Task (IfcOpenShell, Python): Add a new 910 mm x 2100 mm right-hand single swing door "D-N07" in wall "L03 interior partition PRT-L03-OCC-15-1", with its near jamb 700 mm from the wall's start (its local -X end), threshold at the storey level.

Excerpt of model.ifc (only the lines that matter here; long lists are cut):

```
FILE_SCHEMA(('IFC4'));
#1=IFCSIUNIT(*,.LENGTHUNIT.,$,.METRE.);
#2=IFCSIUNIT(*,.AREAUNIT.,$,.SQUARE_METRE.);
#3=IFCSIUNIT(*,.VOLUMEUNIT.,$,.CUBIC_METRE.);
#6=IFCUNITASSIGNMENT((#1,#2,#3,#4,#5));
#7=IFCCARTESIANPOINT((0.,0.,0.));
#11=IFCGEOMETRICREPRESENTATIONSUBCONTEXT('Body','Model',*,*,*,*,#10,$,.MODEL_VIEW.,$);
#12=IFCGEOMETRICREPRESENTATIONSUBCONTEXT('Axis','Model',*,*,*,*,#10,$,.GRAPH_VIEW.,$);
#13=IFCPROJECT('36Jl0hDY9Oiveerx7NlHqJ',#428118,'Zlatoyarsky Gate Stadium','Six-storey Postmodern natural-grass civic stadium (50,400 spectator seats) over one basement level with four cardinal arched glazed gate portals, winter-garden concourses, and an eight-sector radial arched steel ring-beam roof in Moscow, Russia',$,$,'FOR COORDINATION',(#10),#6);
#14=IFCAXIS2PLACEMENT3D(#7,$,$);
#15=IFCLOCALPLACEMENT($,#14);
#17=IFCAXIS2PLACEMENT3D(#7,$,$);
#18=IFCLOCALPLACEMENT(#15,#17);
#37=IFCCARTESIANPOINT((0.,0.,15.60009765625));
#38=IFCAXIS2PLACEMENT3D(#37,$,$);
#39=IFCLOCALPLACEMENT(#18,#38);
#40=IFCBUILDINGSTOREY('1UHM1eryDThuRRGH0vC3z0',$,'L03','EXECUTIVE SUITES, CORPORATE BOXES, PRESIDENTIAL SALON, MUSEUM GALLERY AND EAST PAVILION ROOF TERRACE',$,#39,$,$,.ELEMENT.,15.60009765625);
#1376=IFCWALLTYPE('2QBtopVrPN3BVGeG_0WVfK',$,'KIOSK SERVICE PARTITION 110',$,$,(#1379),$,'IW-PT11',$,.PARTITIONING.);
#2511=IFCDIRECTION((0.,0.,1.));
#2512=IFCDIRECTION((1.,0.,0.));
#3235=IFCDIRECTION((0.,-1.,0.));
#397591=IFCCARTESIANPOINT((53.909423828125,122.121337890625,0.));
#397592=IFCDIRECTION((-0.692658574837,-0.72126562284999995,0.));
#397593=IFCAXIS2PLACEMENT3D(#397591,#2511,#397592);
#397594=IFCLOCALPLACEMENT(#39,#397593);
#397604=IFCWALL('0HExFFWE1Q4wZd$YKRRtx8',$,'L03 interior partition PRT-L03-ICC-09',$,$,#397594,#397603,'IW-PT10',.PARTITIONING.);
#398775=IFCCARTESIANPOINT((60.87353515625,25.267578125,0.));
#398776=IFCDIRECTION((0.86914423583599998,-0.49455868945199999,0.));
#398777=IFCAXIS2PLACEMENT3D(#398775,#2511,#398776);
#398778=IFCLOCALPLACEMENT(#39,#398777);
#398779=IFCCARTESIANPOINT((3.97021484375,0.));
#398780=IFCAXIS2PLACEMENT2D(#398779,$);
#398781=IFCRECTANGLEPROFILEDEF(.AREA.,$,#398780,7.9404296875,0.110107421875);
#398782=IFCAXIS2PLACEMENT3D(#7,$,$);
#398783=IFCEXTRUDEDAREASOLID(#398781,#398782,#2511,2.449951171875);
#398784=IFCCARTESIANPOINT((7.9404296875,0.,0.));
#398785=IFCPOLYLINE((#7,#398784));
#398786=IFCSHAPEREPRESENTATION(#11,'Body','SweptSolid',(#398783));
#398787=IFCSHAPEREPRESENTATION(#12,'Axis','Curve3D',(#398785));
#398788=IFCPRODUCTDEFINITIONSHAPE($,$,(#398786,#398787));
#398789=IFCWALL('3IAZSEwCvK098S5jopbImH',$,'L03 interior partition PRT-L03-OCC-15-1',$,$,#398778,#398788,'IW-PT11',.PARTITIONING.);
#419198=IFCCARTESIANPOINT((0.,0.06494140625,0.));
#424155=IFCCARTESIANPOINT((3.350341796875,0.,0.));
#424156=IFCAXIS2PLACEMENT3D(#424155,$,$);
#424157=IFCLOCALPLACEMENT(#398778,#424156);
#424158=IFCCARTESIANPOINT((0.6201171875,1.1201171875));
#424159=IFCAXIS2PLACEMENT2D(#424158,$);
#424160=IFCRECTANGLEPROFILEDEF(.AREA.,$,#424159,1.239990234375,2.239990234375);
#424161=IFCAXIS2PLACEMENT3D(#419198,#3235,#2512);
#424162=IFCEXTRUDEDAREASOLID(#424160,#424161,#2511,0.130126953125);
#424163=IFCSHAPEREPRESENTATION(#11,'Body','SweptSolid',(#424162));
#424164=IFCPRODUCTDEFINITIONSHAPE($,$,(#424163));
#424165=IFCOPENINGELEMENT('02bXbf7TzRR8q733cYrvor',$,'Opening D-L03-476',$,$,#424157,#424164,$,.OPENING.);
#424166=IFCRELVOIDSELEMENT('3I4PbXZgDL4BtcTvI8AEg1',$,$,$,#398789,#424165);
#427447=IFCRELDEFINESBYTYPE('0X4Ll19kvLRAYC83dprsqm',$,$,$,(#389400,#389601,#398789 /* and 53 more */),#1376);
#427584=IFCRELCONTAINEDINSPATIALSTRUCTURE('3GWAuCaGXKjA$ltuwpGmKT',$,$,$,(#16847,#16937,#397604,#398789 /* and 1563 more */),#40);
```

```python
import numpy as np
import ifcopenshell
import ifcopenshell.api.feature
import ifcopenshell.api.geometry
import ifcopenshell.api.root
import ifcopenshell.api.spatial
import ifcopenshell.geom
import ifcopenshell.util.element
import ifcopenshell.util.placement
import ifcopenshell.util.representation
import ifcopenshell.util.shape
import ifcopenshell.util.unit

model = ifcopenshell.open("model.ifc")
unit_scale = ifcopenshell.util.unit.calculate_unit_scale(model)
settings = ifcopenshell.geom.settings()


def volume(element):
    """Net volume in cubic metres, openings subtracted."""
    shape = ifcopenshell.geom.create_shape(settings, element)
    return ifcopenshell.util.shape.get_volume(shape.geometry)


wall = model.by_guid("3IAZSEwCvK098S5jopbImH")
storey = ifcopenshell.util.element.get_container(wall, ifc_class="IfcBuildingStorey")
context = ifcopenshell.util.representation.get_context(model, "Model", "Body", "MODEL_VIEW")
before = volume(wall)

width, height, from_end, sill = 0.91, 2.1, 0.7, 0.0  # metres

# The wall runs along its own X axis, and the end named is its -X end.
wall_shape = ifcopenshell.geom.create_shape(settings, wall)
x, y, z = ifcopenshell.util.shape.get_vertices(wall_shape.geometry).T
start = x.min() + from_end
face, thickness = float(y.min()), float(y.max() - y.min())
wall_matrix = ifcopenshell.util.placement.get_local_placement(wall.ObjectPlacement)
level = ifcopenshell.util.placement.get_local_placement(storey.ObjectPlacement)[2, 3]


def in_wall(x, y):
    """Placement at x, y metres in the wall's axes, at sill height."""
    matrix = wall_matrix.copy()
    matrix[:, 3] = wall_matrix @ np.array([x / unit_scale, y / unit_scale, 0.0, 1.0])
    matrix[2, 3] = level + sill / unit_scale
    return matrix


# Opening: a box that overshoots both wall faces by 50 mm.
opening = ifcopenshell.api.root.create_entity(model, ifc_class="IfcOpeningElement", predefined_type="OPENING")
box = ifcopenshell.api.geometry.add_wall_representation(
    model, context=context, length=width, height=height, thickness=thickness + 0.1
)
ifcopenshell.api.geometry.assign_representation(model, product=opening, representation=box)
ifcopenshell.api.geometry.edit_object_placement(model, product=opening, matrix=in_wall(start, face - 0.05), is_si=False)
ifcopenshell.api.feature.add_feature(model, feature=opening, element=wall)

door = ifcopenshell.api.root.create_entity(model, ifc_class="IfcDoor", name="D-N07", predefined_type="DOOR")
door.OverallWidth, door.OverallHeight = width / unit_scale, height / unit_scale
door.OperationType = "SINGLE_SWING_RIGHT"
body = ifcopenshell.api.geometry.add_door_representation(
    model,
    context=context,
    overall_width=door.OverallWidth,
    overall_height=door.OverallHeight,
    operation_type="SINGLE_SWING_RIGHT",
    lining_properties={"LiningDepth": thickness / unit_scale, "ThresholdDepth": thickness / unit_scale},
)
ifcopenshell.api.geometry.assign_representation(model, product=door, representation=body)
ifcopenshell.api.spatial.assign_container(model, products=[door], relating_structure=storey)
ifcopenshell.api.feature.add_filling(model, opening=opening, element=door)

# The lining spans the wall, so the door starts at the wall face.
ifcopenshell.api.geometry.edit_object_placement(model, product=door, matrix=in_wall(start, face), is_si=False)

after = volume(wall)

print(f"wall volume {before:.3f} -> {after:.3f} m3")

model.write("model_updated.ifc")
```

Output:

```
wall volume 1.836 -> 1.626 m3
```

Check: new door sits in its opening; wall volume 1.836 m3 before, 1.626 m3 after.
